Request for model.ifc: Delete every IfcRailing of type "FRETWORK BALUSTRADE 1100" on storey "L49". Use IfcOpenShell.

First a look at what the model holds.

```python
import ifcopenshell
import ifcopenshell.util.element

model = ifcopenshell.open("model.ifc")
print(model.schema)
storey = next(s for s in model.by_type("IfcBuildingStorey") if s.Name == "L49")
railings = [e for e in ifcopenshell.util.element.get_decomposition(storey) if e.is_a("IfcRailing")]
seen = {}
for e in railings:
    element_type = ifcopenshell.util.element.get_type(e)
    name = element_type.Name if element_type not in (None, e) else None
    seen[name] = seen.get(name, 0) + 1
for name, count in sorted(seen.items(), key=str):
    print(count, "x", name)
```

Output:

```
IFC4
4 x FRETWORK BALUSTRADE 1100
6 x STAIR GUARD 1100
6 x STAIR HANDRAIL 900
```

```python
import ifcopenshell
import ifcopenshell.api.root
import ifcopenshell.util.element

model = ifcopenshell.open("model.ifc")

storey = next(s for s in model.by_type("IfcBuildingStorey") if s.Name == "L49")
railings = [e for e in ifcopenshell.util.element.get_decomposition(storey) if e.is_a("IfcRailing")]
targets = [e for e in railings if (t := ifcopenshell.util.element.get_type(e)) not in (None, e) and t.Name == "FRETWORK BALUSTRADE 1100"]

for e in targets:
    ifcopenshell.api.root.remove_product(model, product=e)
print(len(targets), "removed")

model.write("model_v2.ifc")
```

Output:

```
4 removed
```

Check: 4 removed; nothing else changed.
